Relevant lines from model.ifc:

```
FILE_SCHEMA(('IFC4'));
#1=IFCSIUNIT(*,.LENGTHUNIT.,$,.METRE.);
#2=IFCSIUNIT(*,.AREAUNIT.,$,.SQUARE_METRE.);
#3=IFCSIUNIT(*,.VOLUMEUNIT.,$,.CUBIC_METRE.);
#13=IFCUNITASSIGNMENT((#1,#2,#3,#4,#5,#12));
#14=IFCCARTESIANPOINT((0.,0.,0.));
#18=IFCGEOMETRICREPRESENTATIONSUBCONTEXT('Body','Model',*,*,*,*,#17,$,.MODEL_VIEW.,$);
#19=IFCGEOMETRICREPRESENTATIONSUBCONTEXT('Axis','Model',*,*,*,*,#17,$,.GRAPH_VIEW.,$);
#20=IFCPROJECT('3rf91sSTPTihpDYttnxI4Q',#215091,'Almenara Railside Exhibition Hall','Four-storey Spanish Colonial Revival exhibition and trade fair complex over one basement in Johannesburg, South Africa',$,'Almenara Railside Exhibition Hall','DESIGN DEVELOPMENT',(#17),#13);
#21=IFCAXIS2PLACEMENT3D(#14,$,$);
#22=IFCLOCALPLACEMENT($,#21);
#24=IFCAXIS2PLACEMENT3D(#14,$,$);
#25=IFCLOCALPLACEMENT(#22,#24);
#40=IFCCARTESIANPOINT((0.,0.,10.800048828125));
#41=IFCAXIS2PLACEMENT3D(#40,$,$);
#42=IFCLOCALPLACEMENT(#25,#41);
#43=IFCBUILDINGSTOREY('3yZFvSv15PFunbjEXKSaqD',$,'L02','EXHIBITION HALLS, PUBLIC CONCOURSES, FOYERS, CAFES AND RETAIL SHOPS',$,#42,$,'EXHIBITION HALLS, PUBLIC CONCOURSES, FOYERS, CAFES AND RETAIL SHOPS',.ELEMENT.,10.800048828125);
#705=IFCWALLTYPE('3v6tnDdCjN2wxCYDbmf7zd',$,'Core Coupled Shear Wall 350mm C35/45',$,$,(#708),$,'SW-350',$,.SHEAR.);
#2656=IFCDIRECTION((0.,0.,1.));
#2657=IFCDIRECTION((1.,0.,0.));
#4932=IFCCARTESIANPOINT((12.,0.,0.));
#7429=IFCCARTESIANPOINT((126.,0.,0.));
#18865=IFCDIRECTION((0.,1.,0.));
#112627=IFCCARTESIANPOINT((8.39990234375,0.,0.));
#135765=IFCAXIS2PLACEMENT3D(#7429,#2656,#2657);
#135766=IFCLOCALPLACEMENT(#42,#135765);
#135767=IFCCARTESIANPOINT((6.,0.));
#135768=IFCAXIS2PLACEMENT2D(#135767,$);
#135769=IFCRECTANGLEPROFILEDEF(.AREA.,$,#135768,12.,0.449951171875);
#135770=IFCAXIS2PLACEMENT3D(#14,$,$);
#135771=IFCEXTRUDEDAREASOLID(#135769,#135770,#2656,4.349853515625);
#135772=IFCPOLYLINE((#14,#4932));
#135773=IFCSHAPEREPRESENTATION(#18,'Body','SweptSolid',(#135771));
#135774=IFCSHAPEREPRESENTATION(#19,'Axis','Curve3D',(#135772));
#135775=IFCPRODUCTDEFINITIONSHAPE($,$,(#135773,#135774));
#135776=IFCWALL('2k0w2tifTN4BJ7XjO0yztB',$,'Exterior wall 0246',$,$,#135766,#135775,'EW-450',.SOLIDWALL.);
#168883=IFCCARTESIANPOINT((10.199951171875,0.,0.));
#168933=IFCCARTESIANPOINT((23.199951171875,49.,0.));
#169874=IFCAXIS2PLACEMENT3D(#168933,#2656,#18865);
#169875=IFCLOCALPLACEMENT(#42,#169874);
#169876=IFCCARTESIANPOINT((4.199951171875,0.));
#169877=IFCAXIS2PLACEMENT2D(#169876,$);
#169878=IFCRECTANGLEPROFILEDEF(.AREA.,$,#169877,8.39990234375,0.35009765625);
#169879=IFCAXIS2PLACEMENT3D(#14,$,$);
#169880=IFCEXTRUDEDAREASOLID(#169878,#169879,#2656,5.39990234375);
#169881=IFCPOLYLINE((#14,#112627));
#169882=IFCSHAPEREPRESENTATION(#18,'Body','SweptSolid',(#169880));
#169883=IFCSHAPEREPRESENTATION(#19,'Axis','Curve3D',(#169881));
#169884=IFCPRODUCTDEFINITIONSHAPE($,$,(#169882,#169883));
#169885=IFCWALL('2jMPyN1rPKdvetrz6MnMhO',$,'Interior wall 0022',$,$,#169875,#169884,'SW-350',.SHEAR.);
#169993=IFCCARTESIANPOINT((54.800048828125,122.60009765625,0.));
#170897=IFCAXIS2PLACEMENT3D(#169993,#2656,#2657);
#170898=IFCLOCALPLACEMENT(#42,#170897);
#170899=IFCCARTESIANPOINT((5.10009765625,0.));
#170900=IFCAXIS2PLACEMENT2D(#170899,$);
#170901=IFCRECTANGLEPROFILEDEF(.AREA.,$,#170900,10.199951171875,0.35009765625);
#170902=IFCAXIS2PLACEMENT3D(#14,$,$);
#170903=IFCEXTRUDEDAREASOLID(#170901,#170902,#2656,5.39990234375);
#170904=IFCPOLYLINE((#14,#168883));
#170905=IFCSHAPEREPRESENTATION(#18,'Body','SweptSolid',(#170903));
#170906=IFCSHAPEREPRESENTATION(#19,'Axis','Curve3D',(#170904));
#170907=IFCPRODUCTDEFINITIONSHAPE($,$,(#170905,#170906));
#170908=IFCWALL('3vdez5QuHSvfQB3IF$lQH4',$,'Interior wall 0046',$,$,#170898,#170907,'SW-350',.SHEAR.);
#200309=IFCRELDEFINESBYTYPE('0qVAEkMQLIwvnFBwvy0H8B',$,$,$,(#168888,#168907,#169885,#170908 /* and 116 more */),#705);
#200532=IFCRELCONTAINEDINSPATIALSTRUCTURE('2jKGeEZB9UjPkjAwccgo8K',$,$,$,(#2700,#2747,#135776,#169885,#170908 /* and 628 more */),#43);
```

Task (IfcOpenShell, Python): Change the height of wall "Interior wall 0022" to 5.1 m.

```python
import ifcopenshell
import ifcopenshell.geom
import ifcopenshell.util.representation
import ifcopenshell.util.shape

model = ifcopenshell.open("model.ifc")
settings = ifcopenshell.geom.settings()


def volume(element):
    """Net volume in cubic metres, openings subtracted."""
    shape = ifcopenshell.geom.create_shape(settings, element)
    return ifcopenshell.util.shape.get_volume(shape.geometry)


wall = model.by_guid("2jMPyN1rPKdvetrz6MnMhO")
before = volume(wall)

body = ifcopenshell.util.representation.get_representation(wall, "Model", "Body")
solid = body.Items[0]
old_height = solid.Depth
solid.Depth = 5.1
after = volume(wall)

print(f"height {old_height:g} -> {solid.Depth:g}, volume {before:.3f} -> {after:.3f} m3")

model.write("model_v2.ifc")
```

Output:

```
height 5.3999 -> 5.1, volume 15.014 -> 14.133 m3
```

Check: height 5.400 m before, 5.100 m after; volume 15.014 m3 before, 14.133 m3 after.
